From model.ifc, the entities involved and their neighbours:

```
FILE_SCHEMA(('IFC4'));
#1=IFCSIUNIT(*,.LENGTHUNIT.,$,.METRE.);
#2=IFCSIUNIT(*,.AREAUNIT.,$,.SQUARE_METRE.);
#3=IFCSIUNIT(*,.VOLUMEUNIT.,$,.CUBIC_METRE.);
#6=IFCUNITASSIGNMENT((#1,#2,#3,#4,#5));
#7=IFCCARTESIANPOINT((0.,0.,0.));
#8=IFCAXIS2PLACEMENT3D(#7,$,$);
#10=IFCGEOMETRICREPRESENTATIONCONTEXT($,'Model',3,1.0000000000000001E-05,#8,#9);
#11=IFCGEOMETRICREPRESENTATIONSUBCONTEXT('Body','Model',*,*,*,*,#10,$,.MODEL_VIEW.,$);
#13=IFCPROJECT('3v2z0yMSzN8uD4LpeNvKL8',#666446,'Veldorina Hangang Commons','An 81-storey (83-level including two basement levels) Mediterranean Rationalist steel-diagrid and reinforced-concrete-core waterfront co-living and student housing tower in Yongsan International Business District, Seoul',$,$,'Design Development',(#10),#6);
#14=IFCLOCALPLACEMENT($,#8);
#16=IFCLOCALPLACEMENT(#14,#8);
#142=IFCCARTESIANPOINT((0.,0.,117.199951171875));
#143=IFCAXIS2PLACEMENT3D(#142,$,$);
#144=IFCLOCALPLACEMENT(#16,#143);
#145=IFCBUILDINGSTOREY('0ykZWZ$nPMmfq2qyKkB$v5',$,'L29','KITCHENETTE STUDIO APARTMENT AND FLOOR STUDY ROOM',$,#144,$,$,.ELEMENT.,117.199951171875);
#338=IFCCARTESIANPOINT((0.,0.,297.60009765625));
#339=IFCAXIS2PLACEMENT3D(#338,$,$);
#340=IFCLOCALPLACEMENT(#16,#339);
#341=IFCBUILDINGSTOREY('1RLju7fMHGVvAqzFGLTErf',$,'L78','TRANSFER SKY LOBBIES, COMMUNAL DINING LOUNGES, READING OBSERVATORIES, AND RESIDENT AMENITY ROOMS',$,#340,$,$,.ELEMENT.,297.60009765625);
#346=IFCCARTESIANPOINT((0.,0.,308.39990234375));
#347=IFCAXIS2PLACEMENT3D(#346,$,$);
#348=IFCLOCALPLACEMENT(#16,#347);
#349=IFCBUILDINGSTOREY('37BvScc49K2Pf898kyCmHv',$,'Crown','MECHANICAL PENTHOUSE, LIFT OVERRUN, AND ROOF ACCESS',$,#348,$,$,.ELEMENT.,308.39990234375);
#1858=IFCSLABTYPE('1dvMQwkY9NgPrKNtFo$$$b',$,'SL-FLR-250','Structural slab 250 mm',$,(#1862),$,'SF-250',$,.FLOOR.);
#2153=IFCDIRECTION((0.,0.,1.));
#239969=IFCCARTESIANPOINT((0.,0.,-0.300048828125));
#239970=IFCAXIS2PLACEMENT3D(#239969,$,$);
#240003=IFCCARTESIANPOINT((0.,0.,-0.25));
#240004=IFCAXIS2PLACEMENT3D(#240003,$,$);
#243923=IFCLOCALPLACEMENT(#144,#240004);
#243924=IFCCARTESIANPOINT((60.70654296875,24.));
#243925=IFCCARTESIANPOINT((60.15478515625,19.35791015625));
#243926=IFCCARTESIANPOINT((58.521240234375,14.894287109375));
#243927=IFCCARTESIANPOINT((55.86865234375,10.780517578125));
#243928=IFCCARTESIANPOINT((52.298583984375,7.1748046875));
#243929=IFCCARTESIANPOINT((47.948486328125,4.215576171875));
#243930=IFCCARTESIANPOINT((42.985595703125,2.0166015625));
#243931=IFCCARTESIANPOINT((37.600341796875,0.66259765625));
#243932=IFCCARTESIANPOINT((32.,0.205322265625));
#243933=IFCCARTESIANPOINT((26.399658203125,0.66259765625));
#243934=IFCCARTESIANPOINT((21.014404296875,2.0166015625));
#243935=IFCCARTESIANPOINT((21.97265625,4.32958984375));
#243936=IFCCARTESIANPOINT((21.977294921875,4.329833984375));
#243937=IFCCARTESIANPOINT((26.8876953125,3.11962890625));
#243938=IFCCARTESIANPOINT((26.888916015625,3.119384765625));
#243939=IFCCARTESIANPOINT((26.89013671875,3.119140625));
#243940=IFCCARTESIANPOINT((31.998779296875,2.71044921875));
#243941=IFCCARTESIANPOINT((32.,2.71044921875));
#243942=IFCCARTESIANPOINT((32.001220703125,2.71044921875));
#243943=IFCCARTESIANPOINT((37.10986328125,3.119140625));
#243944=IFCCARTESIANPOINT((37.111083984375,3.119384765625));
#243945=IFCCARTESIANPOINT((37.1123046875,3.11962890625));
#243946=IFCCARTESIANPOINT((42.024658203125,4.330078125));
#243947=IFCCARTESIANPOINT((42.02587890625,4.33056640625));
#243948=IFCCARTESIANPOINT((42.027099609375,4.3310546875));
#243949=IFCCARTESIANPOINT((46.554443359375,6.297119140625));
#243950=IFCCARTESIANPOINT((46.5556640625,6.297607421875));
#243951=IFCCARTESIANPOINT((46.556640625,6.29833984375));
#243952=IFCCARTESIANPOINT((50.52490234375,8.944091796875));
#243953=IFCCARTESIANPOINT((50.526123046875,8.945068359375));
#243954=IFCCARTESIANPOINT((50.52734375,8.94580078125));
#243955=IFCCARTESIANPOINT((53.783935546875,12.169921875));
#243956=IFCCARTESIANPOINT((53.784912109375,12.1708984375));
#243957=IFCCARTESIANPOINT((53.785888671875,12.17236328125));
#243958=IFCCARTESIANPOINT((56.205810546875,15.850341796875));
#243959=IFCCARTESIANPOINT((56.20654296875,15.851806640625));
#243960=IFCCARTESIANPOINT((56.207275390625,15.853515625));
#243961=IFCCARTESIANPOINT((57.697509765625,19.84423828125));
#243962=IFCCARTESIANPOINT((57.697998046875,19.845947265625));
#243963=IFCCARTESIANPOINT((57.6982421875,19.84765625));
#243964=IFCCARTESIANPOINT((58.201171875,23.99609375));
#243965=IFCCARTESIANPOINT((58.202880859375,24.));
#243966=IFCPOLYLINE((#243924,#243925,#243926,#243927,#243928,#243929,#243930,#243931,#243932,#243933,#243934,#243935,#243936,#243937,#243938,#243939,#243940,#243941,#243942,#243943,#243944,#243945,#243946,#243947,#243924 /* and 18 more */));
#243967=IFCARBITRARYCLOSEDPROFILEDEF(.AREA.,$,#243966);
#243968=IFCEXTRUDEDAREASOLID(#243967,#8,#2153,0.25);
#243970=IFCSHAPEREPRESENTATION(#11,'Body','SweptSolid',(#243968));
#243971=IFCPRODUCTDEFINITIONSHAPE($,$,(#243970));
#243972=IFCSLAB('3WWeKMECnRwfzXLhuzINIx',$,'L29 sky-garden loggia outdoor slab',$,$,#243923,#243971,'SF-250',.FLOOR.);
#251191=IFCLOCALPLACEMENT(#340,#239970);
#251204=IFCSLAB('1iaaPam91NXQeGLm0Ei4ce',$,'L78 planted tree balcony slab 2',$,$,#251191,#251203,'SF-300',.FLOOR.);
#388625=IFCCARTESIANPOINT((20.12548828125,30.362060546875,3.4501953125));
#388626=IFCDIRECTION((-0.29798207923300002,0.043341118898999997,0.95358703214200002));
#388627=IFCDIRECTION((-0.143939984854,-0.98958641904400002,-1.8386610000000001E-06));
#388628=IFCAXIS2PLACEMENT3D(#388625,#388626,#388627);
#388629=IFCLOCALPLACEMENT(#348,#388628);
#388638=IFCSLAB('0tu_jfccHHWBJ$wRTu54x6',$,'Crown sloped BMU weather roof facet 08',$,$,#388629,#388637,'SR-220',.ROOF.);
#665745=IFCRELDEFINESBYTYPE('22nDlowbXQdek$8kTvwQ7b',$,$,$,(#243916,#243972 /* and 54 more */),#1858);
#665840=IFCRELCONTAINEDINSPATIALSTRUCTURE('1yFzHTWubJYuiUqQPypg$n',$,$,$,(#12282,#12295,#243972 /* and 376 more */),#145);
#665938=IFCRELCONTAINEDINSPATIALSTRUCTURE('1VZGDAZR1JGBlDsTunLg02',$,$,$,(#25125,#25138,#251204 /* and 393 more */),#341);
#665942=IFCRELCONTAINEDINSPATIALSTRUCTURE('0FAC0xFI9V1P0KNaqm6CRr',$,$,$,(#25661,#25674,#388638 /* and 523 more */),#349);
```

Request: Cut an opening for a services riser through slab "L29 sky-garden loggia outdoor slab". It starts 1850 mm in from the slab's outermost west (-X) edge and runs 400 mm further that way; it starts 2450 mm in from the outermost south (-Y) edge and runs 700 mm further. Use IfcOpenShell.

```python
import numpy as np
import ifcopenshell
import ifcopenshell.api.feature
import ifcopenshell.api.geometry
import ifcopenshell.api.root
import ifcopenshell.geom
import ifcopenshell.util.placement
import ifcopenshell.util.representation
import ifcopenshell.util.shape
import ifcopenshell.util.unit

model = ifcopenshell.open("model.ifc")
unit_scale = ifcopenshell.util.unit.calculate_unit_scale(model)
settings = ifcopenshell.geom.settings()


def volume(element):
    """Net volume in cubic metres, openings subtracted."""
    shape = ifcopenshell.geom.create_shape(settings, element)
    return ifcopenshell.util.shape.get_volume(shape.geometry)


slab = model.by_guid("3WWeKMECnRwfzXLhuzINIx")
before = volume(slab)

# Extent in the slab's own axes, in metres. The edges named are its -X and -Y sides.
slab_shape = ifcopenshell.geom.create_shape(settings, slab)
vertices = ifcopenshell.util.shape.get_vertices(slab_shape.geometry)
x_min, y_min, bottom = vertices.min(axis=0)
top = vertices[:, 2].max()

opening = ifcopenshell.api.root.create_entity(model, ifc_class="IfcOpeningElement", name="Services riser opening", predefined_type="OPENING")
context = ifcopenshell.util.representation.get_context(model, "Model", "Body", "MODEL_VIEW")
width, depth = 0.4, 0.7
outline = [(0.0, 0.0), (width, 0.0), (width, depth), (0.0, depth), (0.0, 0.0)]
# Overshoot both faces by 50 mm so the cut is clean.
shape = ifcopenshell.api.geometry.add_slab_representation(
    model, context=context, depth=top - bottom + 0.1, polyline=outline
)
ifcopenshell.api.geometry.assign_representation(model, product=opening, representation=shape)

matrix = ifcopenshell.util.placement.get_local_placement(slab.ObjectPlacement)
matrix[:, 3] = matrix @ np.append(np.array([x_min + 1.85, y_min + 2.45, bottom - 0.05]) / unit_scale, 1.0)
ifcopenshell.api.geometry.edit_object_placement(model, product=opening, matrix=matrix, is_si=False)
ifcopenshell.api.feature.add_feature(model, feature=opening, element=slab)

after = volume(slab)

print(f"slab volume {before:.3f} -> {after:.3f} m3")

model.write("model_edited.ifc")
```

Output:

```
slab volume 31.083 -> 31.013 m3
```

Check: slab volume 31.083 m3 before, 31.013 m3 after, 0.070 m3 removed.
